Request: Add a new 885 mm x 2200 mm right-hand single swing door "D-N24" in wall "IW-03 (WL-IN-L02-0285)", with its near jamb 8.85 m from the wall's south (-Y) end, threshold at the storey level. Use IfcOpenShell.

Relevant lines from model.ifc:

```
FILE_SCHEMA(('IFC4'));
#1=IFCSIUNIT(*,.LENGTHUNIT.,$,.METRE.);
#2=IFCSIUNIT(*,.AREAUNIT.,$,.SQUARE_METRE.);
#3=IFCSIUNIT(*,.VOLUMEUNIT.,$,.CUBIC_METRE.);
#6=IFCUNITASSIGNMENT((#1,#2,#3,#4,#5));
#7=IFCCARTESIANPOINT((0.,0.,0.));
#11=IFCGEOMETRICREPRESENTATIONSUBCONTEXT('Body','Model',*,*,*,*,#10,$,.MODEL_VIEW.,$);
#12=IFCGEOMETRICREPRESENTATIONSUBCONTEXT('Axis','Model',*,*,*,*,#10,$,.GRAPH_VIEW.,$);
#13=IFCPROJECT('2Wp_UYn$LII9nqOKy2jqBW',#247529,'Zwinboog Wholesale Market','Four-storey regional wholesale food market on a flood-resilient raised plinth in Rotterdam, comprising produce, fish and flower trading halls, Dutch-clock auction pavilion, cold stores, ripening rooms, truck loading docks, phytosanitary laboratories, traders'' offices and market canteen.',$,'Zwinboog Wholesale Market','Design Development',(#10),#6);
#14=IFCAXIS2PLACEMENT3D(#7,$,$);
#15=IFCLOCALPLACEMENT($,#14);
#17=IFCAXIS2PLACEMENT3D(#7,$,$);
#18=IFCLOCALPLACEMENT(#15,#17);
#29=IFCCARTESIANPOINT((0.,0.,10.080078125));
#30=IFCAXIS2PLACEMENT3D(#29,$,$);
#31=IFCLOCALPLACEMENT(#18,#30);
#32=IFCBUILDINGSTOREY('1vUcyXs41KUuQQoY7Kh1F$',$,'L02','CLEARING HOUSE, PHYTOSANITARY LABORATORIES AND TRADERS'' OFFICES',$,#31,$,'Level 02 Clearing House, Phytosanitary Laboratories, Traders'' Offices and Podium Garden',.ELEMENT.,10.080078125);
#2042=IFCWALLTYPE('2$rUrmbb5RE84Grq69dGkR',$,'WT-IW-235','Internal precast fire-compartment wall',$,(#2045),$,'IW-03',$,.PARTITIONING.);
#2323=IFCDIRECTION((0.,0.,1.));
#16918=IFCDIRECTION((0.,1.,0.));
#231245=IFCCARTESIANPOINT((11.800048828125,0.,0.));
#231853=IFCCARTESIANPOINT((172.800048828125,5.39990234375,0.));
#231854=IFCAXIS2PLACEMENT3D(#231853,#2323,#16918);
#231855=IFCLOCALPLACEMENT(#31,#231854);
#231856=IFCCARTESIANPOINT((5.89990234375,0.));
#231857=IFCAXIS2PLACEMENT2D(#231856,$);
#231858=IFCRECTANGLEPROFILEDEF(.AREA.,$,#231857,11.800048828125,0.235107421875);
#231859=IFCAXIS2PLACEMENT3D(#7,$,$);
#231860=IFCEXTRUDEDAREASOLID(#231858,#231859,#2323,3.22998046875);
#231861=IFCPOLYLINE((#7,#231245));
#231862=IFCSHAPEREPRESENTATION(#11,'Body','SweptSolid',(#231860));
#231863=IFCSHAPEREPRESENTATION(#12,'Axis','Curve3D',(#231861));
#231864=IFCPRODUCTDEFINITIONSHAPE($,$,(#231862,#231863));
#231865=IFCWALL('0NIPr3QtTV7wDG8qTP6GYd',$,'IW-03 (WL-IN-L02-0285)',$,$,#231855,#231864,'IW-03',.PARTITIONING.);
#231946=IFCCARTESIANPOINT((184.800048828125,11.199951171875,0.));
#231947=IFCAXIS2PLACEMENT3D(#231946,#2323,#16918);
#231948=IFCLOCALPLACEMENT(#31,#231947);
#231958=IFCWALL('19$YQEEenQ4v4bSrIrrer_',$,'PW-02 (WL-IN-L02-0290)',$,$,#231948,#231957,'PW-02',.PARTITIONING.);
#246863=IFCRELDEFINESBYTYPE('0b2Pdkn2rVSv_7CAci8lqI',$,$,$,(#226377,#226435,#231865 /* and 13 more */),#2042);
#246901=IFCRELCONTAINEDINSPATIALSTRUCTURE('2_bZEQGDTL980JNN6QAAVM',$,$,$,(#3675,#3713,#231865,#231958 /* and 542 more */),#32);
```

```python
import numpy as np
import ifcopenshell
import ifcopenshell.api.feature
import ifcopenshell.api.geometry
import ifcopenshell.api.root
import ifcopenshell.api.spatial
import ifcopenshell.geom
import ifcopenshell.util.element
import ifcopenshell.util.placement
import ifcopenshell.util.representation
import ifcopenshell.util.shape
import ifcopenshell.util.unit

model = ifcopenshell.open("model.ifc")
unit_scale = ifcopenshell.util.unit.calculate_unit_scale(model)
settings = ifcopenshell.geom.settings()


def volume(element):
    """Net volume in cubic metres, openings subtracted."""
    shape = ifcopenshell.geom.create_shape(settings, element)
    return ifcopenshell.util.shape.get_volume(shape.geometry)


wall = model.by_guid("0NIPr3QtTV7wDG8qTP6GYd")
storey = ifcopenshell.util.element.get_container(wall, ifc_class="IfcBuildingStorey")
context = ifcopenshell.util.representation.get_context(model, "Model", "Body", "MODEL_VIEW")
before = volume(wall)

width, height, from_end, sill = 0.885, 2.2, 8.85, 0.0  # metres

# The wall runs along its own X axis, and the end named is its -X end.
wall_shape = ifcopenshell.geom.create_shape(settings, wall)
x, y, z = ifcopenshell.util.shape.get_vertices(wall_shape.geometry).T
start = x.min() + from_end
face, thickness = float(y.min()), float(y.max() - y.min())
wall_matrix = ifcopenshell.util.placement.get_local_placement(wall.ObjectPlacement)
level = ifcopenshell.util.placement.get_local_placement(storey.ObjectPlacement)[2, 3]


def in_wall(x, y):
    """Placement at x, y metres in the wall's axes, at sill height."""
    matrix = wall_matrix.copy()
    matrix[:, 3] = wall_matrix @ np.array([x / unit_scale, y / unit_scale, 0.0, 1.0])
    matrix[2, 3] = level + sill / unit_scale
    return matrix


# Opening: a box that overshoots both wall faces by 50 mm.
opening = ifcopenshell.api.root.create_entity(model, ifc_class="IfcOpeningElement", predefined_type="OPENING")
box = ifcopenshell.api.geometry.add_wall_representation(
    model, context=context, length=width, height=height, thickness=thickness + 0.1
)
ifcopenshell.api.geometry.assign_representation(model, product=opening, representation=box)
ifcopenshell.api.geometry.edit_object_placement(model, product=opening, matrix=in_wall(start, face - 0.05), is_si=False)
ifcopenshell.api.feature.add_feature(model, feature=opening, element=wall)

door = ifcopenshell.api.root.create_entity(model, ifc_class="IfcDoor", name="D-N24", predefined_type="DOOR")
door.OverallWidth, door.OverallHeight = width / unit_scale, height / unit_scale
door.OperationType = "SINGLE_SWING_RIGHT"
body = ifcopenshell.api.geometry.add_door_representation(
    model,
    context=context,
    overall_width=door.OverallWidth,
    overall_height=door.OverallHeight,
    operation_type="SINGLE_SWING_RIGHT",
    lining_properties={"LiningDepth": thickness / unit_scale, "ThresholdDepth": thickness / unit_scale},
)
ifcopenshell.api.geometry.assign_representation(model, product=door, representation=body)
ifcopenshell.api.spatial.assign_container(model, products=[door], relating_structure=storey)
ifcopenshell.api.feature.add_filling(model, opening=opening, element=door)

# The lining spans the wall, so the door starts at the wall face.
ifcopenshell.api.geometry.edit_object_placement(model, product=door, matrix=in_wall(start, face), is_si=False)

after = volume(wall)

print(f"wall volume {before:.3f} -> {after:.3f} m3")

model.write("model-out.ifc")
```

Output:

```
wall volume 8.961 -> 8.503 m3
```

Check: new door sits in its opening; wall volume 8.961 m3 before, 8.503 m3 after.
